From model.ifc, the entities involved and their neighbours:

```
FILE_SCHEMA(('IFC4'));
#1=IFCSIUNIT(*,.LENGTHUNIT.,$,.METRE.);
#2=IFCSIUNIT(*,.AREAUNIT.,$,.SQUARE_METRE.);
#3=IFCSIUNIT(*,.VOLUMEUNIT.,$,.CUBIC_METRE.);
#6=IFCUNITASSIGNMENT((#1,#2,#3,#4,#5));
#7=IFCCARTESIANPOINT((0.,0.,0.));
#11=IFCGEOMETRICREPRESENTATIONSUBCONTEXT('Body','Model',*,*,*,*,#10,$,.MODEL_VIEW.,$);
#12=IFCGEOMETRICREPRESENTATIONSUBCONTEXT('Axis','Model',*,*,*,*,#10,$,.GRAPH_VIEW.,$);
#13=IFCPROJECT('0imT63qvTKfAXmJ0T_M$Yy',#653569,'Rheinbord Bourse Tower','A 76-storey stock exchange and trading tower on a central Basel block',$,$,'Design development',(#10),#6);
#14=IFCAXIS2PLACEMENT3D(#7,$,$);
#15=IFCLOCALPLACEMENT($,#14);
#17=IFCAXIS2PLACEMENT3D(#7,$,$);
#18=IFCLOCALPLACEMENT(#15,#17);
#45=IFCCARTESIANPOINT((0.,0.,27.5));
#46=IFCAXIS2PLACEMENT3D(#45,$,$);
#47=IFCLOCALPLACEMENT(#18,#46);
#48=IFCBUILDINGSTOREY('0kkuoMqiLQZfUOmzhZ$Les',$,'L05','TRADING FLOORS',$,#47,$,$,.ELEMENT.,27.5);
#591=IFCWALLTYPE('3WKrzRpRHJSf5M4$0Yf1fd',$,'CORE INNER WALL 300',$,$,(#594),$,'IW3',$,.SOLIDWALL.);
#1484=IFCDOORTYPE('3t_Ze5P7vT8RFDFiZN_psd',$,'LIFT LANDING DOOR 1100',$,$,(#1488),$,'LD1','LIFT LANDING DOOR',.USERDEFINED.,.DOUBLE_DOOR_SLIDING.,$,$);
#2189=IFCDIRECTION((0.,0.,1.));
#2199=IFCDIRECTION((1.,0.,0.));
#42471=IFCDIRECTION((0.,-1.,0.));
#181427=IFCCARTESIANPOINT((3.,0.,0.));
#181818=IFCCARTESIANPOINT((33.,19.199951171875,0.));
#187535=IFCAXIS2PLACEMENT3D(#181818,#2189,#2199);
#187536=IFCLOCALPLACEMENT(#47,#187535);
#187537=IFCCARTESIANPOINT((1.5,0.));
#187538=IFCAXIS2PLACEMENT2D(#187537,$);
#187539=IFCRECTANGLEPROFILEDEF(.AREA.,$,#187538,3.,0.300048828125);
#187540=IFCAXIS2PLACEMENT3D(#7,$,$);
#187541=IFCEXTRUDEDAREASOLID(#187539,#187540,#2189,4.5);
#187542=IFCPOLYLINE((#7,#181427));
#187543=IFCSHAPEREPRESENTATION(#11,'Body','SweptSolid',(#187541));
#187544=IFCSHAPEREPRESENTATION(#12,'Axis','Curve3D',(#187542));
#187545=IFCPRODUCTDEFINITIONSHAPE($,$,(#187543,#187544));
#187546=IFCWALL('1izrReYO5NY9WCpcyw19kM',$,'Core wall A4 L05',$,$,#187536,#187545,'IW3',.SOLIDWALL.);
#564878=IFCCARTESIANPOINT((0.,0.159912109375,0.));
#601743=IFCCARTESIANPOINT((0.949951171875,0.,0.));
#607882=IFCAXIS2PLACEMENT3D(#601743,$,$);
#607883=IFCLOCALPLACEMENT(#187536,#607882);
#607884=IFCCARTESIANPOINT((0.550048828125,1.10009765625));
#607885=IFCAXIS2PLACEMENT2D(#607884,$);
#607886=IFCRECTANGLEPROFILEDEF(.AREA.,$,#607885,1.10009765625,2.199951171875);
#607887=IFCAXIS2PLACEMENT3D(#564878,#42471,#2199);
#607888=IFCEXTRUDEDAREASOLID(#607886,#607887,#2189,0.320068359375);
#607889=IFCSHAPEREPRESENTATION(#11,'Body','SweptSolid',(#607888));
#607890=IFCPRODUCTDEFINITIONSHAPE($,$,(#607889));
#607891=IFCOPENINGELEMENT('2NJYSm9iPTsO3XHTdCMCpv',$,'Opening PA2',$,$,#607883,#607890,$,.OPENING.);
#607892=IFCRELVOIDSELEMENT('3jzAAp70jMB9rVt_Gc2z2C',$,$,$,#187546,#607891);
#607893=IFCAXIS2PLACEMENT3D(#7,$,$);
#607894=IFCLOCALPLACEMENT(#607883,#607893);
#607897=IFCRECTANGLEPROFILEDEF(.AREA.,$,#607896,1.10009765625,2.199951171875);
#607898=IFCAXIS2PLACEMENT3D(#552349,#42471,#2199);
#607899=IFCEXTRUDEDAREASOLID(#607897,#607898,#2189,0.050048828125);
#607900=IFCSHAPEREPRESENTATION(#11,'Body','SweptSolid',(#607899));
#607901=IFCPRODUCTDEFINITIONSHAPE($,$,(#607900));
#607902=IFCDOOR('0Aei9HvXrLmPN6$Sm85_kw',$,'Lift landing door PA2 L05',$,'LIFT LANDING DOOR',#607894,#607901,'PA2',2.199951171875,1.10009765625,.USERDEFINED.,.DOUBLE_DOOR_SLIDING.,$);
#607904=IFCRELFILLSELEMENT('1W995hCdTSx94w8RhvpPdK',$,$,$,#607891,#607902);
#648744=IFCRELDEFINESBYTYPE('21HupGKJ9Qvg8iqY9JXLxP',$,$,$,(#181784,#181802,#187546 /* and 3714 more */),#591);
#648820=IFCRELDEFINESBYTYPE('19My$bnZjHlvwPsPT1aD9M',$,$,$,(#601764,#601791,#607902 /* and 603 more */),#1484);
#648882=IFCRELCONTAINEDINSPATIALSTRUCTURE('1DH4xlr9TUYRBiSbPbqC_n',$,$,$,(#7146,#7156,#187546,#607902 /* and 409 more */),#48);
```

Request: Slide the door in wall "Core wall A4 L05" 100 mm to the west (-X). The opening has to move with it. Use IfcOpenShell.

```python
import ifcopenshell
import ifcopenshell.api.geometry
import ifcopenshell.util.placement
import ifcopenshell.util.unit

model = ifcopenshell.open("model.ifc")
unit_scale = ifcopenshell.util.unit.calculate_unit_scale(model)

door = model.by_id(607902)
opening = door.FillsVoids[0].RelatingOpeningElement
wall = opening.VoidsElements[0].RelatingBuildingElement

wall_matrix = ifcopenshell.util.placement.get_local_placement(wall.ObjectPlacement)
shift = wall_matrix[:3, 0] * -0.1 / unit_scale
before = ifcopenshell.util.placement.get_local_placement(door.ObjectPlacement)[:3, 3].copy()

# The door is placed relative to its opening, so it follows when the opening moves.
matrix = ifcopenshell.util.placement.get_local_placement(opening.ObjectPlacement)
matrix[:3, 3] += shift
ifcopenshell.api.geometry.edit_object_placement(
    model, product=opening, matrix=matrix, is_si=False, should_transform_children=True
)

after = ifcopenshell.util.placement.get_local_placement(door.ObjectPlacement)[:3, 3]
print("door moved by", (after - before).round(3) + 0.0)

model.write("model_v2.ifc")
```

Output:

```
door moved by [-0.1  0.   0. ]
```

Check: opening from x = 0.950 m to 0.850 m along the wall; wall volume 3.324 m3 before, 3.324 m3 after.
